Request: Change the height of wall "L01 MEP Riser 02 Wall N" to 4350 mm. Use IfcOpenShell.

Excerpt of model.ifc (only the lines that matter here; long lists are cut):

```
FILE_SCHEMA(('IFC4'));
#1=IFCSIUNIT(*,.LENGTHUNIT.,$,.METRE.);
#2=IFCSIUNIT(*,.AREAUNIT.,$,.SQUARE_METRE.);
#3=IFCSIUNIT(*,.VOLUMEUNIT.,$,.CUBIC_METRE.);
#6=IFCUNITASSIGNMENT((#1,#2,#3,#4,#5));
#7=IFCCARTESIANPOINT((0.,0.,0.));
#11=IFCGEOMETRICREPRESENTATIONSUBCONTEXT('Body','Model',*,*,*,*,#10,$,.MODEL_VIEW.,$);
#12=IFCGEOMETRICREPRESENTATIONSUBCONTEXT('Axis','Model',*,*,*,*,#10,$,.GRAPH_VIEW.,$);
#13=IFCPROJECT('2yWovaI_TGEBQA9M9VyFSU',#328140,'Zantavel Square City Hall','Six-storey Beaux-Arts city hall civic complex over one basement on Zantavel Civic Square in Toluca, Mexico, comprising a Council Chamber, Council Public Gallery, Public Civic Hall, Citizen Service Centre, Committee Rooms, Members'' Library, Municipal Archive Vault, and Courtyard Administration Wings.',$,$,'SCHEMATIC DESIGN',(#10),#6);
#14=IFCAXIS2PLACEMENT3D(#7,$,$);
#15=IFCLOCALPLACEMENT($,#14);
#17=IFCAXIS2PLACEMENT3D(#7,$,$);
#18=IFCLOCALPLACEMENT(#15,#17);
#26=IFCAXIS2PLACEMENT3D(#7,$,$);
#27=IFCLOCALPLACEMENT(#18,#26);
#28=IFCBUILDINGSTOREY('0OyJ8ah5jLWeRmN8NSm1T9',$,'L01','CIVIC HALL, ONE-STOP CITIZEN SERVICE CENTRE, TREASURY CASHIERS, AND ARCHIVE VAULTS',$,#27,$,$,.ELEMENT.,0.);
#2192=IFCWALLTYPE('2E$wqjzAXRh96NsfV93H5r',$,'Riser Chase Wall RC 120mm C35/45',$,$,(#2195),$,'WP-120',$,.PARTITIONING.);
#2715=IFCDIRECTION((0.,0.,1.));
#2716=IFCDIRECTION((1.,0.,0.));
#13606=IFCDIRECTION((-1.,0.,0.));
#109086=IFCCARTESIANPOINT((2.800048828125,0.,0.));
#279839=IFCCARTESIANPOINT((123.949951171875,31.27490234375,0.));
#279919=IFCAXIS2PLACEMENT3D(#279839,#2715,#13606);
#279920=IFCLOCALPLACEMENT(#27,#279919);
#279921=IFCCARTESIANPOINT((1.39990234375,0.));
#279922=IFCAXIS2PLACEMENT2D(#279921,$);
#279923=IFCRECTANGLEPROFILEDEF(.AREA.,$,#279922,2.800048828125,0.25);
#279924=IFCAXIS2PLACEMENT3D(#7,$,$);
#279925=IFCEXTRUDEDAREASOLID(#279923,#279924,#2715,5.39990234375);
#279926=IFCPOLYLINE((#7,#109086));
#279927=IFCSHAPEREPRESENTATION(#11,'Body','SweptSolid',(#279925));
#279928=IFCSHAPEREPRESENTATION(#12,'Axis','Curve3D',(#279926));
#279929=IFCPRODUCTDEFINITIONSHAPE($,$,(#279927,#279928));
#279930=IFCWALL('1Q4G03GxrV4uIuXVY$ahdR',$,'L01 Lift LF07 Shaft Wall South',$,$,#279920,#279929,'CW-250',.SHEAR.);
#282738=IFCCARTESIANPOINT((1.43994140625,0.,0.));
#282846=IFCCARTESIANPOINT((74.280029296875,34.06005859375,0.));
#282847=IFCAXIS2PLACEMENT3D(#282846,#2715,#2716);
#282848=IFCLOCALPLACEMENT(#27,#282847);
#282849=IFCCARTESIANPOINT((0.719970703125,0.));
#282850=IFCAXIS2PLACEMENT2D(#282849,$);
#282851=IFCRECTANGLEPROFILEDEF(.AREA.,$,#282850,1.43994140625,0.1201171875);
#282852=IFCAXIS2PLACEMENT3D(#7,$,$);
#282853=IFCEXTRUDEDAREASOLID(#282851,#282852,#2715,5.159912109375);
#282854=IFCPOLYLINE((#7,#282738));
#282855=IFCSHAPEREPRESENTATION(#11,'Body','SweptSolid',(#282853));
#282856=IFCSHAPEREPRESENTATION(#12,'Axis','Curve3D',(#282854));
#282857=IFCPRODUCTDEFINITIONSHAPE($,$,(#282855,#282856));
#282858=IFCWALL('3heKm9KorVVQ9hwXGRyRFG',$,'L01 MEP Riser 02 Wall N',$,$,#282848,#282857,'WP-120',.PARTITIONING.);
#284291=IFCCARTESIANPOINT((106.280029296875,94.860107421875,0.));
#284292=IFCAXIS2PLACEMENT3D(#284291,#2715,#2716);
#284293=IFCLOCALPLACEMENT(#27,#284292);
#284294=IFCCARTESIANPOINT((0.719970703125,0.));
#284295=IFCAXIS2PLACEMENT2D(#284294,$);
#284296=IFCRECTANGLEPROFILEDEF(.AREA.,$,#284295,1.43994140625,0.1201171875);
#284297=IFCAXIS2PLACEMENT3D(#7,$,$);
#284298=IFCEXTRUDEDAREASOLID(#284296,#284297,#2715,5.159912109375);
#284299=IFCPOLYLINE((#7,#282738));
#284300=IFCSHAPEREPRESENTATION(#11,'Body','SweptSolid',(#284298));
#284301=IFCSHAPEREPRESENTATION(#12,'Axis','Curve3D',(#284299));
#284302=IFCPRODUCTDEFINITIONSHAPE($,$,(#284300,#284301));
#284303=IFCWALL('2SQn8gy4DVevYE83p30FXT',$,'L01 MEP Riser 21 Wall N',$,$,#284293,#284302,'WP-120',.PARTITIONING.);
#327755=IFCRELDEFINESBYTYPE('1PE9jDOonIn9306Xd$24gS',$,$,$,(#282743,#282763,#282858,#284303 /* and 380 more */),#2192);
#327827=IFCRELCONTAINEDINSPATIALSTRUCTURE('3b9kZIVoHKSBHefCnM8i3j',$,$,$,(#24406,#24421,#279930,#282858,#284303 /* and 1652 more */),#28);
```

```python
import ifcopenshell
import ifcopenshell.geom
import ifcopenshell.util.representation
import ifcopenshell.util.shape

model = ifcopenshell.open("model.ifc")
settings = ifcopenshell.geom.settings()


def volume(element):
    """Net volume in cubic metres, openings subtracted."""
    shape = ifcopenshell.geom.create_shape(settings, element)
    return ifcopenshell.util.shape.get_volume(shape.geometry)


wall = model.by_id(282858)
before = volume(wall)

body = ifcopenshell.util.representation.get_representation(wall, "Model", "Body")
solid = body.Items[0]
old_height = solid.Depth
solid.Depth = 4.35
after = volume(wall)

print(f"height {old_height:g} -> {solid.Depth:g}, volume {before:.3f} -> {after:.3f} m3")

model.write("model_updated.ifc")
```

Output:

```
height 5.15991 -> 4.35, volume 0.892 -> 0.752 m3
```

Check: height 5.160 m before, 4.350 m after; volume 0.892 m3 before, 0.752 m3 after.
